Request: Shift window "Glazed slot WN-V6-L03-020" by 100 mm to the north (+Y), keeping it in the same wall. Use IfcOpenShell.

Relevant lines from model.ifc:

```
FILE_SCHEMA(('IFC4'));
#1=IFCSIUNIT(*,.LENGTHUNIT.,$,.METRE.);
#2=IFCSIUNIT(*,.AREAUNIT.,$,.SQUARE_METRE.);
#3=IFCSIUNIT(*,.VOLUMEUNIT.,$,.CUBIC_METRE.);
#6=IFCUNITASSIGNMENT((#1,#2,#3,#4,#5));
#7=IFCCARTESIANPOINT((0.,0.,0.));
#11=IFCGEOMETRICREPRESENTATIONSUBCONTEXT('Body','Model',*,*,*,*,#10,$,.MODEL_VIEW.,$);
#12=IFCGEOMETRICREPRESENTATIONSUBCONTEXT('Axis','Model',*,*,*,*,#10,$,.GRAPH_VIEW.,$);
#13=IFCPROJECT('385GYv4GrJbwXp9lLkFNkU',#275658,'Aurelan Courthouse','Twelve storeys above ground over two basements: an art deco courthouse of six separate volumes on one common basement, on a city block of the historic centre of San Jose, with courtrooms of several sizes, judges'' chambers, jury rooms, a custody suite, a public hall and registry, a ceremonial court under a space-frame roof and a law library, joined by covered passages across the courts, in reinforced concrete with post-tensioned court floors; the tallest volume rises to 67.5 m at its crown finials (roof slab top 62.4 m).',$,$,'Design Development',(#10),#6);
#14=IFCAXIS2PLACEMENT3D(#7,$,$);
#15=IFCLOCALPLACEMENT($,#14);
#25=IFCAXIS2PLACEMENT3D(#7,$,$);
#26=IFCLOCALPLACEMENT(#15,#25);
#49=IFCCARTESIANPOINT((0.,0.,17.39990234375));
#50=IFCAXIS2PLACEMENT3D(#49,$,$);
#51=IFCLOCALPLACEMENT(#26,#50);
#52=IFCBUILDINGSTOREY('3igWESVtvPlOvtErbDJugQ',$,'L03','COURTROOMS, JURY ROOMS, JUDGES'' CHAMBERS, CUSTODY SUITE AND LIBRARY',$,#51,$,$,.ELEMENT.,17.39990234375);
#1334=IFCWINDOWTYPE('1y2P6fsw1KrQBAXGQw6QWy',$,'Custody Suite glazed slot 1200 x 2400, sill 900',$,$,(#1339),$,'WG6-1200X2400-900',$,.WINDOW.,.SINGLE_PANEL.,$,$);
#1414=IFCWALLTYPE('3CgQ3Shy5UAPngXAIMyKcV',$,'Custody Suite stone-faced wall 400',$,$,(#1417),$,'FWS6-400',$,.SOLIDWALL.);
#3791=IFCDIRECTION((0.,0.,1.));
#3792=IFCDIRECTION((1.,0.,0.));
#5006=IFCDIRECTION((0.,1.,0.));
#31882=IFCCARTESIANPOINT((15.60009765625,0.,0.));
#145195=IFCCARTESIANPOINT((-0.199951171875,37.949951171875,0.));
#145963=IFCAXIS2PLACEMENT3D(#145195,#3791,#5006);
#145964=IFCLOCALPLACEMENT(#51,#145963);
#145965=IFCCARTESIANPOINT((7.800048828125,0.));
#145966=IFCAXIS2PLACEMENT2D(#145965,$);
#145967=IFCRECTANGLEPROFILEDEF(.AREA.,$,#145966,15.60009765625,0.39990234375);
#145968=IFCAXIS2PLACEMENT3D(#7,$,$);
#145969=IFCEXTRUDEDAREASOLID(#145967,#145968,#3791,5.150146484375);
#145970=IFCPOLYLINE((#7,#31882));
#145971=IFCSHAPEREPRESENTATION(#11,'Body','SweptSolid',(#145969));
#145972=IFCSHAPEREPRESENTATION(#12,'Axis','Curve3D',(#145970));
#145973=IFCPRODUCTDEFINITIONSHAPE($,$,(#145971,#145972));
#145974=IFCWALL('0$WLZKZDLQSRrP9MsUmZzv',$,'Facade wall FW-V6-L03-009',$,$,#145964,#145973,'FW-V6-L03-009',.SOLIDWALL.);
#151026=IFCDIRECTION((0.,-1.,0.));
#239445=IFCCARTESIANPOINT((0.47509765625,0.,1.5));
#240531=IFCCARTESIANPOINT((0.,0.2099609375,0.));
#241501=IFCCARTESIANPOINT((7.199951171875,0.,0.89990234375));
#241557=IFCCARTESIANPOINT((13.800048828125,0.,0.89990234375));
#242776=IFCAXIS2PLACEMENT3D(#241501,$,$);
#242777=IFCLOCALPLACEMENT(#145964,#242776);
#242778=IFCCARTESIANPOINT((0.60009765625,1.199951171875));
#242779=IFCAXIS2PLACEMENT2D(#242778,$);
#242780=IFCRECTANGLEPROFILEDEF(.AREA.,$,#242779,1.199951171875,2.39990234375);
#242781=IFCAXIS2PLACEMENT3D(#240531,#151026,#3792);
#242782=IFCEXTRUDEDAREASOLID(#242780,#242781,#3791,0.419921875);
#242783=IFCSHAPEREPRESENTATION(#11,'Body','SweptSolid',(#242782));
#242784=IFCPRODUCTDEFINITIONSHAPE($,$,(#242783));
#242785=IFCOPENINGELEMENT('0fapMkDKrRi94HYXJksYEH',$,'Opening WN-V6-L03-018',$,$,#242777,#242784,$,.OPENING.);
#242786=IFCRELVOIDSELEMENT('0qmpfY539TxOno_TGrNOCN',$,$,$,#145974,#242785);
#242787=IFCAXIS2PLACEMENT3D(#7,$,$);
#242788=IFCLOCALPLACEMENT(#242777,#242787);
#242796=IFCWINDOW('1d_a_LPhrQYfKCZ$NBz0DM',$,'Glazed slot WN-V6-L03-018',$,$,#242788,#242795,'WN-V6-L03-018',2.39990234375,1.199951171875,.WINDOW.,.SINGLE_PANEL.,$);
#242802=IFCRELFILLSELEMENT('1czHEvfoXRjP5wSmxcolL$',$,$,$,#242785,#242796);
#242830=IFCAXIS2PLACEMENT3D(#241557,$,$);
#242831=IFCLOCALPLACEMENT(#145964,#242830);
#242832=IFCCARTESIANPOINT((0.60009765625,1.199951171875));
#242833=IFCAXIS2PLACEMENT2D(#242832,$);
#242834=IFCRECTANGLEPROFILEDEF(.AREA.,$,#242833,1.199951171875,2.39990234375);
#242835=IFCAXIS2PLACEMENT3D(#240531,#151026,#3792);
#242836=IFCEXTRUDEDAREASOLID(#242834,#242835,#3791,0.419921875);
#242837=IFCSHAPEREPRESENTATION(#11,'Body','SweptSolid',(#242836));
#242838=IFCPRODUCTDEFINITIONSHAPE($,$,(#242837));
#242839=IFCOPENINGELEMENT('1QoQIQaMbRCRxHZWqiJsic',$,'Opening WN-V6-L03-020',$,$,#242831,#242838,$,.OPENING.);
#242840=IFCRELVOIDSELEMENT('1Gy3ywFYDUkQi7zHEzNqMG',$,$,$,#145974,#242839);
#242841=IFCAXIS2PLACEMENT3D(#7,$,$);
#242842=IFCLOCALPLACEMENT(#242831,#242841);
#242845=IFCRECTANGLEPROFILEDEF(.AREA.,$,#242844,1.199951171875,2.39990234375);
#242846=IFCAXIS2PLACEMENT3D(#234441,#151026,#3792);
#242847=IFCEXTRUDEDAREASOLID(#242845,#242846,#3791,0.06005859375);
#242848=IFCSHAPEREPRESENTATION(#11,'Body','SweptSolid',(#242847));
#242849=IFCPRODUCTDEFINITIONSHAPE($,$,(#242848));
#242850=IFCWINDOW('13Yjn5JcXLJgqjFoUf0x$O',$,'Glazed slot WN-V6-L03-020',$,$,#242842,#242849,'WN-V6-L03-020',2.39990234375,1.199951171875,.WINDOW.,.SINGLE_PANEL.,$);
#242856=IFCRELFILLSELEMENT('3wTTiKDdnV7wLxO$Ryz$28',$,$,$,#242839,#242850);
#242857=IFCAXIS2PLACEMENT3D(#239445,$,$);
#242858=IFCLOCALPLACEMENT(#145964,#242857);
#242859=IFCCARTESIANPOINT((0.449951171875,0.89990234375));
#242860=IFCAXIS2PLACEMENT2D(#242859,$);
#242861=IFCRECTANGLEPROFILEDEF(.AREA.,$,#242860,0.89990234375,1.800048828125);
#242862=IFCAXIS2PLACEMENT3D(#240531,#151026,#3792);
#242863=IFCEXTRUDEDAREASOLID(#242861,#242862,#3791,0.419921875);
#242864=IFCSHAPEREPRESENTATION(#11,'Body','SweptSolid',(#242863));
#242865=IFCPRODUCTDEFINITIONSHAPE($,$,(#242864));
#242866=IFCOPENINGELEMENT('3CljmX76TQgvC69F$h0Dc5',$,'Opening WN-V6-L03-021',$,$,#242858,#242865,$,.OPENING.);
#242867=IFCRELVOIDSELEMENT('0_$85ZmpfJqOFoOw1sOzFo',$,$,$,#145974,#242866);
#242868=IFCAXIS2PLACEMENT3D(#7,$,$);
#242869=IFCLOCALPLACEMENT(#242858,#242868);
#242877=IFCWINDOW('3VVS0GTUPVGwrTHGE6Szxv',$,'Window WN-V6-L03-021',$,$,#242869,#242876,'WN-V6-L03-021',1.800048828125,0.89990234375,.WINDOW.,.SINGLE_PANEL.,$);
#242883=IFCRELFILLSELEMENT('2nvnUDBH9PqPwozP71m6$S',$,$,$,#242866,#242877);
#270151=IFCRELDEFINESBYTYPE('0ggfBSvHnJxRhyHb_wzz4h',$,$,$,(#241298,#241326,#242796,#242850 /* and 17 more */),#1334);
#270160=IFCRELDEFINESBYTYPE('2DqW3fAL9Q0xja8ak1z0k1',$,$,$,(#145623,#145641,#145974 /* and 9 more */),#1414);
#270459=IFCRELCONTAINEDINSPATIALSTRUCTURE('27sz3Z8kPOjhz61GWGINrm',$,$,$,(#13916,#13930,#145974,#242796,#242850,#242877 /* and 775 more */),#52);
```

```python
import ifcopenshell
import ifcopenshell.api.geometry
import ifcopenshell.util.placement
import ifcopenshell.util.unit

model = ifcopenshell.open("model.ifc")
unit_scale = ifcopenshell.util.unit.calculate_unit_scale(model)

window = model.by_guid("13Yjn5JcXLJgqjFoUf0x$O")
opening = window.FillsVoids[0].RelatingOpeningElement
wall = opening.VoidsElements[0].RelatingBuildingElement

wall_matrix = ifcopenshell.util.placement.get_local_placement(wall.ObjectPlacement)
shift = wall_matrix[:3, 0] * 0.1 / unit_scale
before = ifcopenshell.util.placement.get_local_placement(window.ObjectPlacement)[:3, 3].copy()

# The window is placed relative to its opening, so it follows when the opening moves.
matrix = ifcopenshell.util.placement.get_local_placement(opening.ObjectPlacement)
matrix[:3, 3] += shift
ifcopenshell.api.geometry.edit_object_placement(
    model, product=opening, matrix=matrix, is_si=False, should_transform_children=True
)

after = ifcopenshell.util.placement.get_local_placement(window.ObjectPlacement)[:3, 3]
print("window moved by", (after - before).round(3) + 0.0)

model.write("model-out.ifc")
```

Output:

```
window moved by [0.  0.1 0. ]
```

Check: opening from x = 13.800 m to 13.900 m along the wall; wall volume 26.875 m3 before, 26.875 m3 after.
